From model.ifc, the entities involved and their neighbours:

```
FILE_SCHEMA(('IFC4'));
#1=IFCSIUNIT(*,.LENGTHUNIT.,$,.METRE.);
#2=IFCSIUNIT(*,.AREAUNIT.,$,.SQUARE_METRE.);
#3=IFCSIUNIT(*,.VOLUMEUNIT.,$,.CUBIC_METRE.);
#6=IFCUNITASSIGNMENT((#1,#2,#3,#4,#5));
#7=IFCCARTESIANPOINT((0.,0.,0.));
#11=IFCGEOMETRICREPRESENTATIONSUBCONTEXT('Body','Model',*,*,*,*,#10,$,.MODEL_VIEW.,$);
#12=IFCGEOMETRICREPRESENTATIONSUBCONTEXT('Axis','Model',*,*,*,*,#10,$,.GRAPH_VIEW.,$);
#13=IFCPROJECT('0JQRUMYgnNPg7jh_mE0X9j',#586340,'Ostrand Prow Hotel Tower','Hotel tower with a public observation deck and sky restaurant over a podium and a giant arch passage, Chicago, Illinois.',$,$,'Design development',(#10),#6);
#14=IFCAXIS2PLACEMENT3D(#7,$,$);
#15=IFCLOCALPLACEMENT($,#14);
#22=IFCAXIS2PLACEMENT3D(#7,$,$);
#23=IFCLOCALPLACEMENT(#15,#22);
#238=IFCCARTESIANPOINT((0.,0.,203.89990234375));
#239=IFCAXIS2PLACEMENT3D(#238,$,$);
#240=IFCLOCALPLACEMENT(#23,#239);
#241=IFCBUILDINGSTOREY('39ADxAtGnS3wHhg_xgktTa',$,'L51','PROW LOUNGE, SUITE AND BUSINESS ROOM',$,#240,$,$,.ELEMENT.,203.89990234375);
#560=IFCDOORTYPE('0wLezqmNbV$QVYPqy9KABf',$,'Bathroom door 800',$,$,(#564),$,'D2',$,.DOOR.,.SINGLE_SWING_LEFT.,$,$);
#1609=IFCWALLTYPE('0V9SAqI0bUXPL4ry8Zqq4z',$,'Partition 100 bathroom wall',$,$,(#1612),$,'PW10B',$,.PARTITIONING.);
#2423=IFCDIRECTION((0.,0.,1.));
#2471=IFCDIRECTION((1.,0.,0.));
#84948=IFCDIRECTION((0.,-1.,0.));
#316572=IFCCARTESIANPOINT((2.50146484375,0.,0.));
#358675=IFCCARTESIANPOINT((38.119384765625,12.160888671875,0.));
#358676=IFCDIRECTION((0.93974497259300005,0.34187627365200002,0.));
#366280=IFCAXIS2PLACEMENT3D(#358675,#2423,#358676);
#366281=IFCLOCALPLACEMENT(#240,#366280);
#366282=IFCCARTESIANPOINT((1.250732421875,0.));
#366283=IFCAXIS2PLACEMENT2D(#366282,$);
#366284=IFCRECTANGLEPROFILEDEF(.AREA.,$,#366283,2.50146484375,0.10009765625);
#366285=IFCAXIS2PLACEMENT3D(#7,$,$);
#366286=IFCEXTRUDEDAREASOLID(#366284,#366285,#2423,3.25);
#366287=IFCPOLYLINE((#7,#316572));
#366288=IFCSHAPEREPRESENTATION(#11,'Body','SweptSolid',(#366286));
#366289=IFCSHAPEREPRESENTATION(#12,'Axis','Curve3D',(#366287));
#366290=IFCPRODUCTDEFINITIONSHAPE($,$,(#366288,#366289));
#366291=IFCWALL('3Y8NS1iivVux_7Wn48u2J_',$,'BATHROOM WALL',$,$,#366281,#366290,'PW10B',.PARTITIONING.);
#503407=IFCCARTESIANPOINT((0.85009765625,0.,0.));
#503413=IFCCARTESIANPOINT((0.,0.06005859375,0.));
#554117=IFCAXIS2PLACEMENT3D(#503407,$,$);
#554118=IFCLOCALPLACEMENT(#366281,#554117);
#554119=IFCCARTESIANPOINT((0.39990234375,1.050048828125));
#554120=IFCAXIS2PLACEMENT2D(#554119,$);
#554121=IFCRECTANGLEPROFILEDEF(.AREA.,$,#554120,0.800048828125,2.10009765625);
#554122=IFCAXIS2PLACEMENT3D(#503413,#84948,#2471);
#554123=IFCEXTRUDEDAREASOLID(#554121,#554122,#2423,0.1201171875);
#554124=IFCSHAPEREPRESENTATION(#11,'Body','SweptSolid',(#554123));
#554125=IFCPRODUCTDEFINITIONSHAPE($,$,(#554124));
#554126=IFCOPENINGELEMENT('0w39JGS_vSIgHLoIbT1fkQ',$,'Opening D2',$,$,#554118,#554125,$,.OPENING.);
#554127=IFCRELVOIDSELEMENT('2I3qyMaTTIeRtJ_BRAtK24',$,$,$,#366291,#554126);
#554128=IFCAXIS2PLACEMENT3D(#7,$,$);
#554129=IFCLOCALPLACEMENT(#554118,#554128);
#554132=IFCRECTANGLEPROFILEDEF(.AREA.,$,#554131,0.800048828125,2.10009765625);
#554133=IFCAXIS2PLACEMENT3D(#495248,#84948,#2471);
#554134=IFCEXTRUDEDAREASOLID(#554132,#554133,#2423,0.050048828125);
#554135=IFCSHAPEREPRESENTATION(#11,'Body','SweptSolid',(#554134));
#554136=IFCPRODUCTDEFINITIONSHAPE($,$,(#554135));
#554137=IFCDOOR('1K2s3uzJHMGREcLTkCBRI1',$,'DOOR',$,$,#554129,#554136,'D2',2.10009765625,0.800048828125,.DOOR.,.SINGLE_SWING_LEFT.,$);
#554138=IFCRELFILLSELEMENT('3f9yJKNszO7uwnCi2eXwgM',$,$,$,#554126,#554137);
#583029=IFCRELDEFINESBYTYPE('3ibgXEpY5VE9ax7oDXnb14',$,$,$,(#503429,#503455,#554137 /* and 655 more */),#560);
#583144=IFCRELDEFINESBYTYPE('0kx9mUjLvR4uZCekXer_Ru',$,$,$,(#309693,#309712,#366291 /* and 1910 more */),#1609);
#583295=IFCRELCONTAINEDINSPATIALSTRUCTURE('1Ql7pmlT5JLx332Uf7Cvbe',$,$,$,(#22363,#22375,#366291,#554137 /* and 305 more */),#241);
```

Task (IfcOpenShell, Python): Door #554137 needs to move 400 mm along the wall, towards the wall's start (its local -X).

```python
import ifcopenshell
import ifcopenshell.api.geometry
import ifcopenshell.util.placement

model = ifcopenshell.open("model.ifc")

door = model.by_guid("1K2s3uzJHMGREcLTkCBRI1")
opening = door.FillsVoids[0].RelatingOpeningElement
wall = opening.VoidsElements[0].RelatingBuildingElement

wall_matrix = ifcopenshell.util.placement.get_local_placement(wall.ObjectPlacement)
shift = wall_matrix[:3, 0] * -0.4
before = ifcopenshell.util.placement.get_local_placement(door.ObjectPlacement)[:3, 3].copy()

# The door is placed relative to its opening, so it follows when the opening moves.
matrix = ifcopenshell.util.placement.get_local_placement(opening.ObjectPlacement)
matrix[:3, 3] += shift
ifcopenshell.api.geometry.edit_object_placement(
    model, product=opening, matrix=matrix, is_si=False, should_transform_children=True
)

after = ifcopenshell.util.placement.get_local_placement(door.ObjectPlacement)[:3, 3]
print("door moved by", (after - before).round(3) + 0.0)

model.write("model_v2.ifc")
```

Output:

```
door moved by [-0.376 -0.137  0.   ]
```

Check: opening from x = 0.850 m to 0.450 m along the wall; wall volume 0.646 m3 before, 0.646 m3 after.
